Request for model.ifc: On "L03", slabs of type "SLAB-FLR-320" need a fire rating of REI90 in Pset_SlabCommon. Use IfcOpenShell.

First a look at what the model holds.

```python
import ifcopenshell
import ifcopenshell.util.element

model = ifcopenshell.open("model.ifc")
print(model.schema)
storey = next(s for s in model.by_type("IfcBuildingStorey") if s.Name == "L03")
slabs = [e for e in ifcopenshell.util.element.get_decomposition(storey) if e.is_a("IfcSlab")]
seen = {}
for e in slabs:
    element_type = ifcopenshell.util.element.get_type(e)
    key = (element_type.Name if element_type != e and element_type else None, ifcopenshell.util.element.get_pset(e, "Pset_SlabCommon", "FireRating"))
    seen[key] = seen.get(key, 0) + 1
for (name, value), count in sorted(seen.items(), key=str):
    print(count, "x", name, "|", value)
```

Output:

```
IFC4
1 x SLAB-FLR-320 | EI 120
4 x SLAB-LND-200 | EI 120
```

```python
import ifcopenshell
import ifcopenshell.api.pset
import ifcopenshell.util.element

model = ifcopenshell.open("model.ifc")

storey = next(s for s in model.by_type("IfcBuildingStorey") if s.Name == "L03")
slabs = [e for e in ifcopenshell.util.element.get_decomposition(storey) if e.is_a("IfcSlab")]

count = 0
for e in slabs:
    element_type = ifcopenshell.util.element.get_type(e)
    if element_type in (None, e) or element_type.Name != "SLAB-FLR-320":
        continue
    found = ifcopenshell.util.element.get_pset(e, "Pset_SlabCommon", should_inherit=False)
    if found:
        pset = model.by_id(found["id"])
        if len(ifcopenshell.util.element.get_elements_by_pset(pset)) > 1:
            pset = ifcopenshell.api.pset.unshare_pset(model, products=[e], pset=pset)[0]
    else:
        pset = ifcopenshell.api.pset.add_pset(model, product=e, name="Pset_SlabCommon")
    ifcopenshell.api.pset.edit_pset(model, pset=pset, properties={"FireRating": "REI90"})
    count += 1

print(count, "slabs updated")

model.write("model_updated.ifc")
```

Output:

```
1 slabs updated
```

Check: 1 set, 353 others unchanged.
